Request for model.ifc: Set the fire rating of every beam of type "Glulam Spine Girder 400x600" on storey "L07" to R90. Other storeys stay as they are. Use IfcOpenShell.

First a look at what the model holds.

```python
import ifcopenshell
import ifcopenshell.util.element

model = ifcopenshell.open("model.ifc")
print(model.schema)
storey = next(s for s in model.by_type("IfcBuildingStorey") if s.Name == "L07")
beams = [e for e in ifcopenshell.util.element.get_decomposition(storey) if e.is_a("IfcBeam")]
seen = {}
for e in beams:
    element_type = ifcopenshell.util.element.get_type(e)
    key = (element_type.Name if element_type != e and element_type else None, ifcopenshell.util.element.get_pset(e, "Pset_BeamCommon", "FireRating"))
    seen[key] = seen.get(key, 0) + 1
for (name, value), count in sorted(seen.items(), key=str):
    print(count, "x", name, "|", value)
```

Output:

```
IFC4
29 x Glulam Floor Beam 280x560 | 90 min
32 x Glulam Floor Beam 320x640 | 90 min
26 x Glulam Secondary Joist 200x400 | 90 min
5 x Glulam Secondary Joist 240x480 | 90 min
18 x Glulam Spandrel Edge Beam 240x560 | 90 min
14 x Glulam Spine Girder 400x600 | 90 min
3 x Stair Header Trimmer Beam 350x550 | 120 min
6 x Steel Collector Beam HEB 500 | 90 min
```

```python
import ifcopenshell
import ifcopenshell.api.pset
import ifcopenshell.util.element

model = ifcopenshell.open("model.ifc")

storey = next(s for s in model.by_type("IfcBuildingStorey") if s.Name == "L07")
beams = [e for e in ifcopenshell.util.element.get_decomposition(storey) if e.is_a("IfcBeam")]

count = 0
for e in beams:
    element_type = ifcopenshell.util.element.get_type(e)
    if element_type in (None, e) or element_type.Name != "Glulam Spine Girder 400x600":
        continue
    # add_pset returns the element's existing set when there is one.
    pset = ifcopenshell.api.pset.add_pset(model, product=e, name="Pset_BeamCommon")
    ifcopenshell.api.pset.edit_pset(model, pset=pset, properties={"FireRating": "R90"})
    count += 1

print(count, "beams updated")

model.write("model_rev.ifc")
```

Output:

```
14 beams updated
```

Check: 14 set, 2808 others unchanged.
